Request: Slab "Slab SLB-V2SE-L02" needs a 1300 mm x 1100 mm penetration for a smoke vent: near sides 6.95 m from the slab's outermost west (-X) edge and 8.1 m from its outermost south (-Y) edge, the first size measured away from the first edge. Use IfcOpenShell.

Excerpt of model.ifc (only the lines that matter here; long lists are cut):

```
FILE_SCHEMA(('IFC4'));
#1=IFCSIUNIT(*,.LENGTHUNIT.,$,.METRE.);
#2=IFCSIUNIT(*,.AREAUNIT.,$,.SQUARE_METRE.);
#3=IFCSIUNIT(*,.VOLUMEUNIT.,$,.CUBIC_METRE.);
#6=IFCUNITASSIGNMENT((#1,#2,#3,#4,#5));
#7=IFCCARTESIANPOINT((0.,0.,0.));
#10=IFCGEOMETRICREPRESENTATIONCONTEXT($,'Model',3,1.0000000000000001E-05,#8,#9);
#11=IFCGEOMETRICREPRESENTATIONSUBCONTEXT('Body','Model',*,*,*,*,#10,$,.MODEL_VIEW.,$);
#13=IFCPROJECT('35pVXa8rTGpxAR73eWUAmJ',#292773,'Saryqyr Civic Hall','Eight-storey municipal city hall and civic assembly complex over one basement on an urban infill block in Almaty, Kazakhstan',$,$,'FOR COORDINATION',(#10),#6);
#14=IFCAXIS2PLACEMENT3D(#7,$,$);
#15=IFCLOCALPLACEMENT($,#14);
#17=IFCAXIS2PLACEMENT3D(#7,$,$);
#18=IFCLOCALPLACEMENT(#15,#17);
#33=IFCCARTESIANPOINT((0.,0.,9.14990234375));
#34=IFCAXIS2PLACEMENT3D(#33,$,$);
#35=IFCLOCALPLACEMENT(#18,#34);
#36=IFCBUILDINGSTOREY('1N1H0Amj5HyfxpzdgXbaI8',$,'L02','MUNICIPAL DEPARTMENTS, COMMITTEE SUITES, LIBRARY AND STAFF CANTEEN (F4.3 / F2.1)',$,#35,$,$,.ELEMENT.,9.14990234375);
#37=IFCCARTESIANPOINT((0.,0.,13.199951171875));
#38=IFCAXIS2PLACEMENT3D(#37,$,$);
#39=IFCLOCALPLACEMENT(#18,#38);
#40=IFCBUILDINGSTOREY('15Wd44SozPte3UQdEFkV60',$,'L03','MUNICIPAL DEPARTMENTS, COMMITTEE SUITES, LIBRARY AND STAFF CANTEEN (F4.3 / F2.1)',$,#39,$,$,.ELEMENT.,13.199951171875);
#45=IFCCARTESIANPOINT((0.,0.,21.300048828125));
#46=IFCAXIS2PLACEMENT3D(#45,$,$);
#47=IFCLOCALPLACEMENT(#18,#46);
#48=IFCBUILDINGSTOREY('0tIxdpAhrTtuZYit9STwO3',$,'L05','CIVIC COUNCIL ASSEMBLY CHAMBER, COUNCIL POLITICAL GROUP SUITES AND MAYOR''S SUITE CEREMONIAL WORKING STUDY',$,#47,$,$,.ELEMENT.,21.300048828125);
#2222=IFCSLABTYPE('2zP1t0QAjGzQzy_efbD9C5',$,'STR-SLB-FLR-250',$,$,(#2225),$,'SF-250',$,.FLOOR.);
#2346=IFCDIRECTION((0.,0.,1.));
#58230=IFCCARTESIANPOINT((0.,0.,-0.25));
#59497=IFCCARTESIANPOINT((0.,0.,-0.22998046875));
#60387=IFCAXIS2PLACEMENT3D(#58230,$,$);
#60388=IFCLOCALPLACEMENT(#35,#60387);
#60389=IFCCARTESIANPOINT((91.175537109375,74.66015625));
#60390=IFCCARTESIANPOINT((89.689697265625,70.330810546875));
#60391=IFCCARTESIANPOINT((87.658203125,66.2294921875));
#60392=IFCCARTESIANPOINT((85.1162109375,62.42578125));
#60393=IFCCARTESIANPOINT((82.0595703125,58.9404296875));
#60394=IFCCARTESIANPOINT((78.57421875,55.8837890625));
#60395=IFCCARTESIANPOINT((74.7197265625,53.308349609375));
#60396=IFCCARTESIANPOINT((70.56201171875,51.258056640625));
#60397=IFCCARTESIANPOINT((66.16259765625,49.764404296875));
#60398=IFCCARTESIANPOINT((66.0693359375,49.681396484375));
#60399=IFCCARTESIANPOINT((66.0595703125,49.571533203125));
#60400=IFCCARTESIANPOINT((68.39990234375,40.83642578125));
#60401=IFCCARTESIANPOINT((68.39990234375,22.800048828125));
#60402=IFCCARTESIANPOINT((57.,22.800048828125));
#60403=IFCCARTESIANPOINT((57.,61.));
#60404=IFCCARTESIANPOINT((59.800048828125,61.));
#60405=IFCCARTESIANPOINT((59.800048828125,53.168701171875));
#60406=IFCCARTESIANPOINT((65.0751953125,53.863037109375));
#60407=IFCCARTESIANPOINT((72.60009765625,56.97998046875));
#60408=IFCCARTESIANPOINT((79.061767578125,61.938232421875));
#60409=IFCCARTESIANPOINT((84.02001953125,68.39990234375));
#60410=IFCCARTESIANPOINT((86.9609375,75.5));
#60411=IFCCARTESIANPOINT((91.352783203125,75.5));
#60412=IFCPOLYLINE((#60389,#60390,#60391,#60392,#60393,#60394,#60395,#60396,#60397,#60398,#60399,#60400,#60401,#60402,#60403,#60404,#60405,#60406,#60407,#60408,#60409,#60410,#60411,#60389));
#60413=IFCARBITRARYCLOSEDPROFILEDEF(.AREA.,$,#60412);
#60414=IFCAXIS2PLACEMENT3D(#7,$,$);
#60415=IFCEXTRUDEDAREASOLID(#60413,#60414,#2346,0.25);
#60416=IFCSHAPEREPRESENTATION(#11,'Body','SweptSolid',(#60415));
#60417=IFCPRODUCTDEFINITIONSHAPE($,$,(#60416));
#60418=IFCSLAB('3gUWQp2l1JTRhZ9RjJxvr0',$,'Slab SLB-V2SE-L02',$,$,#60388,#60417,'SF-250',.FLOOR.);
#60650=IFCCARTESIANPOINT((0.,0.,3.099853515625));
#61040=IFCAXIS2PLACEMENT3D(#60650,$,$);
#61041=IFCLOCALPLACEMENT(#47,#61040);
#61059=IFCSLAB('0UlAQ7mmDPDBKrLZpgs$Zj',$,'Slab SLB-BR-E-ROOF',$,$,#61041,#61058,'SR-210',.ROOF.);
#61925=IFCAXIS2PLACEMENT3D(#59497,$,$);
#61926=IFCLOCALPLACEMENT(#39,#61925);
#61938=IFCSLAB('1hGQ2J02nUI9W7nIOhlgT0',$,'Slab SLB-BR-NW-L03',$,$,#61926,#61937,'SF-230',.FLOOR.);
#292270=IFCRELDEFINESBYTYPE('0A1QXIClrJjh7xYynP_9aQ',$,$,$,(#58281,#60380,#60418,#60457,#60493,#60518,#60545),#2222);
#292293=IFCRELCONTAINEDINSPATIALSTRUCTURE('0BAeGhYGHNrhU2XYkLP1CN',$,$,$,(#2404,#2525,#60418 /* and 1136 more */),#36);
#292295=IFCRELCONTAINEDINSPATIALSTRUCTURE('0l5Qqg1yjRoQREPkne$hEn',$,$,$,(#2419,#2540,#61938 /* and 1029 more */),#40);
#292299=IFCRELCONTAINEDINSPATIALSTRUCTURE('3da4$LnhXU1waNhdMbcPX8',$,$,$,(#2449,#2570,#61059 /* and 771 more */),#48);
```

```python
import numpy as np
import ifcopenshell
import ifcopenshell.api.feature
import ifcopenshell.api.geometry
import ifcopenshell.api.root
import ifcopenshell.geom
import ifcopenshell.util.placement
import ifcopenshell.util.representation
import ifcopenshell.util.shape
import ifcopenshell.util.unit

model = ifcopenshell.open("model.ifc")
unit_scale = ifcopenshell.util.unit.calculate_unit_scale(model)
settings = ifcopenshell.geom.settings()


def volume(element):
    """Net volume in cubic metres, openings subtracted."""
    shape = ifcopenshell.geom.create_shape(settings, element)
    return ifcopenshell.util.shape.get_volume(shape.geometry)


slab = model.by_id(60418)
before = volume(slab)

# Extent in the slab's own axes, in metres. The edges named are its -X and -Y sides.
slab_shape = ifcopenshell.geom.create_shape(settings, slab)
vertices = ifcopenshell.util.shape.get_vertices(slab_shape.geometry)
x_min, y_min, bottom = vertices.min(axis=0)
top = vertices[:, 2].max()

opening = ifcopenshell.api.root.create_entity(model, ifc_class="IfcOpeningElement", name="Smoke vent opening", predefined_type="OPENING")
context = ifcopenshell.util.representation.get_context(model, "Model", "Body", "MODEL_VIEW")
width, depth = 1.3, 1.1
outline = [(0.0, 0.0), (width, 0.0), (width, depth), (0.0, depth), (0.0, 0.0)]
# Overshoot both faces by 50 mm so the cut is clean.
shape = ifcopenshell.api.geometry.add_slab_representation(
    model, context=context, depth=top - bottom + 0.1, polyline=outline
)
ifcopenshell.api.geometry.assign_representation(model, product=opening, representation=shape)

matrix = ifcopenshell.util.placement.get_local_placement(slab.ObjectPlacement)
matrix[:, 3] = matrix @ np.append(np.array([x_min + 6.95, y_min + 8.1, bottom - 0.05]) / unit_scale, 1.0)
ifcopenshell.api.geometry.edit_object_placement(model, product=opening, matrix=matrix, is_si=False)
ifcopenshell.api.feature.add_feature(model, feature=opening, element=slab)

after = volume(slab)

print(f"slab volume {before:.3f} -> {after:.3f} m3")

model.write("model-out.ifc")
```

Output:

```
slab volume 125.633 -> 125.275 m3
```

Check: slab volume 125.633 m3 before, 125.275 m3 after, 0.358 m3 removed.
